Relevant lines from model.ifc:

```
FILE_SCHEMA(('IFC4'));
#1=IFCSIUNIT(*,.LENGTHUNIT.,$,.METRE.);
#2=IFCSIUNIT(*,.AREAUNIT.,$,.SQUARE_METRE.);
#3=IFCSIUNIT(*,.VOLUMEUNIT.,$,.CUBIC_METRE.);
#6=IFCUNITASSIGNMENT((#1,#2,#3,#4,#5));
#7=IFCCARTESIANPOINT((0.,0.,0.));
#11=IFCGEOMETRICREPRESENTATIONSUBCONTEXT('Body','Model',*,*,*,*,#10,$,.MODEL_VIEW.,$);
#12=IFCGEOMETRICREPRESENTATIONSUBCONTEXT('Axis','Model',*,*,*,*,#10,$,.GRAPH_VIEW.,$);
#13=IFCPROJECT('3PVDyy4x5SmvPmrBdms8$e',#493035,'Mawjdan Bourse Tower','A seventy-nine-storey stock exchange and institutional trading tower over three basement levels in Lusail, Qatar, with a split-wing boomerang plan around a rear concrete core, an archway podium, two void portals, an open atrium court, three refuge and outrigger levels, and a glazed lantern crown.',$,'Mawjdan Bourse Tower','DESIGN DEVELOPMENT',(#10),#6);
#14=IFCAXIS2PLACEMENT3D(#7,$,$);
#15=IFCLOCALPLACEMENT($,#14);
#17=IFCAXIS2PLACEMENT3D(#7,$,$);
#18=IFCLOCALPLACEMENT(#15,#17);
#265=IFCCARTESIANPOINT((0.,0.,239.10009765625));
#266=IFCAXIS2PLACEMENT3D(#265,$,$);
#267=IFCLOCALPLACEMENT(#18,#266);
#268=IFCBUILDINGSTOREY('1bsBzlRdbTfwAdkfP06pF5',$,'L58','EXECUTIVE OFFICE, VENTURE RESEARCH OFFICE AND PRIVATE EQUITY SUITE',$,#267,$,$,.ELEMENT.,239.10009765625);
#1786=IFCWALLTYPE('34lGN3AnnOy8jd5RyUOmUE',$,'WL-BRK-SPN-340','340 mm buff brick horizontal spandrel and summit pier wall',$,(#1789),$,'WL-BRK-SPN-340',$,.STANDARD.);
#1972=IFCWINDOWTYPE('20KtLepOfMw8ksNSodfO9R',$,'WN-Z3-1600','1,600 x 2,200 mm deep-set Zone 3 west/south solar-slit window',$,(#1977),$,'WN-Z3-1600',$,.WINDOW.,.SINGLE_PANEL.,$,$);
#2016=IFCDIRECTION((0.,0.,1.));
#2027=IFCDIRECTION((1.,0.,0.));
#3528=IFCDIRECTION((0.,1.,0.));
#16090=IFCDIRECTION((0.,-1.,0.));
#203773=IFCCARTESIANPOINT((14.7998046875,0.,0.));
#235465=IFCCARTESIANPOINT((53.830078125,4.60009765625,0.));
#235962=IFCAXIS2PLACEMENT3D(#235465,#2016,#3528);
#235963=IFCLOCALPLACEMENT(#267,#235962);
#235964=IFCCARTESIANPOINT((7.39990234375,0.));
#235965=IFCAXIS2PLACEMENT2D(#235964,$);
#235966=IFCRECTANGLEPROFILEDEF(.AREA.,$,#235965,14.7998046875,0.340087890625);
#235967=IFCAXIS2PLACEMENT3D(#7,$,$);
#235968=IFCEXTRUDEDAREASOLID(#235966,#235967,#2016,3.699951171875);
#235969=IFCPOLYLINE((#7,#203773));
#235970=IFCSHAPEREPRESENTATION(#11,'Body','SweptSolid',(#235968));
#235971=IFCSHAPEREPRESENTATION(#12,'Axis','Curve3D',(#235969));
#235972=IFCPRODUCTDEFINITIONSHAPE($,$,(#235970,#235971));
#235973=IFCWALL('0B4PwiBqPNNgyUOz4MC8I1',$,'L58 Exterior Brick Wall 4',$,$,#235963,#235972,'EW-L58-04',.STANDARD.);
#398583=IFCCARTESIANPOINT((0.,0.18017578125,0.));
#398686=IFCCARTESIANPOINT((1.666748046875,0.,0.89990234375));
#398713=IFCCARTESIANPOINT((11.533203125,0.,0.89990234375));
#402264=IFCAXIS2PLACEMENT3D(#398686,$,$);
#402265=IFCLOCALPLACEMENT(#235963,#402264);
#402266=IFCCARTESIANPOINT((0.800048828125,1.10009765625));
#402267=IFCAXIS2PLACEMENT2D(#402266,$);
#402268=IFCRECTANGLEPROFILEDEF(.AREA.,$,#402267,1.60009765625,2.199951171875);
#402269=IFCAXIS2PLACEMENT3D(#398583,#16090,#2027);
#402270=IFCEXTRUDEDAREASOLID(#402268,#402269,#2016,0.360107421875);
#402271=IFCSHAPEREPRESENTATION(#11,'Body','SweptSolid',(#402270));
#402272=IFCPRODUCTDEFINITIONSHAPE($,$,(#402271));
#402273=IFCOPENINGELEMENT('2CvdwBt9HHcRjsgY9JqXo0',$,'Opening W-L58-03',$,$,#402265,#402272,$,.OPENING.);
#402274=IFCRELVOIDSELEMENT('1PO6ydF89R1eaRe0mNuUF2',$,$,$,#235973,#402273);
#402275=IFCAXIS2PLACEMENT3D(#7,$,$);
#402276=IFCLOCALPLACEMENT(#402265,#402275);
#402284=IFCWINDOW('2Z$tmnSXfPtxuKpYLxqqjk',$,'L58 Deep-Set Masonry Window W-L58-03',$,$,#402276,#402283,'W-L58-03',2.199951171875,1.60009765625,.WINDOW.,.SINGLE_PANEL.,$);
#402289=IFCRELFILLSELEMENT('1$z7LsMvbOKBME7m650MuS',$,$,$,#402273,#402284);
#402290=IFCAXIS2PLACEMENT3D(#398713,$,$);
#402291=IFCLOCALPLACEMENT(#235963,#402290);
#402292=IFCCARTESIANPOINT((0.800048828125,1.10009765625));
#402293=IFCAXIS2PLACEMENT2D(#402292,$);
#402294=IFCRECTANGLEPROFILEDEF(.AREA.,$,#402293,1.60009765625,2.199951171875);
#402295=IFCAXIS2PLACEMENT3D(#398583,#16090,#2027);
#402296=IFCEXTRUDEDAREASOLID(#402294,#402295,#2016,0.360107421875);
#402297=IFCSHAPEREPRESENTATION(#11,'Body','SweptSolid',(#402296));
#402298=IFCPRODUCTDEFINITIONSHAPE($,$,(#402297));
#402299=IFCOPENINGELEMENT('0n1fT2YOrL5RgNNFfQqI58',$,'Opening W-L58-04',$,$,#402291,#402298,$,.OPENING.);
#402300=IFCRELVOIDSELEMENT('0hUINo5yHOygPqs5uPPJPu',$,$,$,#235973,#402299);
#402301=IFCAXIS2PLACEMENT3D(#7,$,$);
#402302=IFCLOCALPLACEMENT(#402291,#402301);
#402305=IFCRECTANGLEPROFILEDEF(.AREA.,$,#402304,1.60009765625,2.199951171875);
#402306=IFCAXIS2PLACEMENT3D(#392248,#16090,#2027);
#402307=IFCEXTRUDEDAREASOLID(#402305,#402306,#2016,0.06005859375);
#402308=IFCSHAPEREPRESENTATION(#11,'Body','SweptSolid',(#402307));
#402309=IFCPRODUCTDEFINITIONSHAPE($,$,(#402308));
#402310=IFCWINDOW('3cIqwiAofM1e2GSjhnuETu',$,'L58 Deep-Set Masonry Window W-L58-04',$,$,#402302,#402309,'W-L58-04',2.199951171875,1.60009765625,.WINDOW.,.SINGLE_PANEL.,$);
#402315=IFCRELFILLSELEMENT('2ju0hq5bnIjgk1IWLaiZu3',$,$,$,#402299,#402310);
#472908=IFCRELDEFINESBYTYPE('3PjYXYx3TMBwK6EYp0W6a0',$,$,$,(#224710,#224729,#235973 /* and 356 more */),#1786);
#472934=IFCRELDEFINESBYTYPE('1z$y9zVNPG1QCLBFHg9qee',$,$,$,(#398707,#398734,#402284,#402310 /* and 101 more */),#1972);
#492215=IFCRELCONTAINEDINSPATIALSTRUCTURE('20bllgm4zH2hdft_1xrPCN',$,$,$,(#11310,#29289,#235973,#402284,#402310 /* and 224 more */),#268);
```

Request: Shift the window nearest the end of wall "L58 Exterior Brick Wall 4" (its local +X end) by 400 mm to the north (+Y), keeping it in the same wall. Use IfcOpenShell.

```python
import ifcopenshell
import ifcopenshell.api.geometry
import ifcopenshell.util.placement

model = ifcopenshell.open("model.ifc")

window = model.by_guid("3cIqwiAofM1e2GSjhnuETu")
opening = window.FillsVoids[0].RelatingOpeningElement
wall = opening.VoidsElements[0].RelatingBuildingElement

wall_matrix = ifcopenshell.util.placement.get_local_placement(wall.ObjectPlacement)
shift = wall_matrix[:3, 0] * 0.4
before = ifcopenshell.util.placement.get_local_placement(window.ObjectPlacement)[:3, 3].copy()

# The window is placed relative to its opening, so it follows when the opening moves.
matrix = ifcopenshell.util.placement.get_local_placement(opening.ObjectPlacement)
matrix[:3, 3] += shift
ifcopenshell.api.geometry.edit_object_placement(
    model, product=opening, matrix=matrix, is_si=False, should_transform_children=True
)

after = ifcopenshell.util.placement.get_local_placement(window.ObjectPlacement)[:3, 3]
print("window moved by", (after - before).round(3) + 0.0)

model.write("model-out.ifc")
```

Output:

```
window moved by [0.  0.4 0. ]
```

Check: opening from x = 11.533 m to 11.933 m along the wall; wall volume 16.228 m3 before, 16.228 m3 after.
